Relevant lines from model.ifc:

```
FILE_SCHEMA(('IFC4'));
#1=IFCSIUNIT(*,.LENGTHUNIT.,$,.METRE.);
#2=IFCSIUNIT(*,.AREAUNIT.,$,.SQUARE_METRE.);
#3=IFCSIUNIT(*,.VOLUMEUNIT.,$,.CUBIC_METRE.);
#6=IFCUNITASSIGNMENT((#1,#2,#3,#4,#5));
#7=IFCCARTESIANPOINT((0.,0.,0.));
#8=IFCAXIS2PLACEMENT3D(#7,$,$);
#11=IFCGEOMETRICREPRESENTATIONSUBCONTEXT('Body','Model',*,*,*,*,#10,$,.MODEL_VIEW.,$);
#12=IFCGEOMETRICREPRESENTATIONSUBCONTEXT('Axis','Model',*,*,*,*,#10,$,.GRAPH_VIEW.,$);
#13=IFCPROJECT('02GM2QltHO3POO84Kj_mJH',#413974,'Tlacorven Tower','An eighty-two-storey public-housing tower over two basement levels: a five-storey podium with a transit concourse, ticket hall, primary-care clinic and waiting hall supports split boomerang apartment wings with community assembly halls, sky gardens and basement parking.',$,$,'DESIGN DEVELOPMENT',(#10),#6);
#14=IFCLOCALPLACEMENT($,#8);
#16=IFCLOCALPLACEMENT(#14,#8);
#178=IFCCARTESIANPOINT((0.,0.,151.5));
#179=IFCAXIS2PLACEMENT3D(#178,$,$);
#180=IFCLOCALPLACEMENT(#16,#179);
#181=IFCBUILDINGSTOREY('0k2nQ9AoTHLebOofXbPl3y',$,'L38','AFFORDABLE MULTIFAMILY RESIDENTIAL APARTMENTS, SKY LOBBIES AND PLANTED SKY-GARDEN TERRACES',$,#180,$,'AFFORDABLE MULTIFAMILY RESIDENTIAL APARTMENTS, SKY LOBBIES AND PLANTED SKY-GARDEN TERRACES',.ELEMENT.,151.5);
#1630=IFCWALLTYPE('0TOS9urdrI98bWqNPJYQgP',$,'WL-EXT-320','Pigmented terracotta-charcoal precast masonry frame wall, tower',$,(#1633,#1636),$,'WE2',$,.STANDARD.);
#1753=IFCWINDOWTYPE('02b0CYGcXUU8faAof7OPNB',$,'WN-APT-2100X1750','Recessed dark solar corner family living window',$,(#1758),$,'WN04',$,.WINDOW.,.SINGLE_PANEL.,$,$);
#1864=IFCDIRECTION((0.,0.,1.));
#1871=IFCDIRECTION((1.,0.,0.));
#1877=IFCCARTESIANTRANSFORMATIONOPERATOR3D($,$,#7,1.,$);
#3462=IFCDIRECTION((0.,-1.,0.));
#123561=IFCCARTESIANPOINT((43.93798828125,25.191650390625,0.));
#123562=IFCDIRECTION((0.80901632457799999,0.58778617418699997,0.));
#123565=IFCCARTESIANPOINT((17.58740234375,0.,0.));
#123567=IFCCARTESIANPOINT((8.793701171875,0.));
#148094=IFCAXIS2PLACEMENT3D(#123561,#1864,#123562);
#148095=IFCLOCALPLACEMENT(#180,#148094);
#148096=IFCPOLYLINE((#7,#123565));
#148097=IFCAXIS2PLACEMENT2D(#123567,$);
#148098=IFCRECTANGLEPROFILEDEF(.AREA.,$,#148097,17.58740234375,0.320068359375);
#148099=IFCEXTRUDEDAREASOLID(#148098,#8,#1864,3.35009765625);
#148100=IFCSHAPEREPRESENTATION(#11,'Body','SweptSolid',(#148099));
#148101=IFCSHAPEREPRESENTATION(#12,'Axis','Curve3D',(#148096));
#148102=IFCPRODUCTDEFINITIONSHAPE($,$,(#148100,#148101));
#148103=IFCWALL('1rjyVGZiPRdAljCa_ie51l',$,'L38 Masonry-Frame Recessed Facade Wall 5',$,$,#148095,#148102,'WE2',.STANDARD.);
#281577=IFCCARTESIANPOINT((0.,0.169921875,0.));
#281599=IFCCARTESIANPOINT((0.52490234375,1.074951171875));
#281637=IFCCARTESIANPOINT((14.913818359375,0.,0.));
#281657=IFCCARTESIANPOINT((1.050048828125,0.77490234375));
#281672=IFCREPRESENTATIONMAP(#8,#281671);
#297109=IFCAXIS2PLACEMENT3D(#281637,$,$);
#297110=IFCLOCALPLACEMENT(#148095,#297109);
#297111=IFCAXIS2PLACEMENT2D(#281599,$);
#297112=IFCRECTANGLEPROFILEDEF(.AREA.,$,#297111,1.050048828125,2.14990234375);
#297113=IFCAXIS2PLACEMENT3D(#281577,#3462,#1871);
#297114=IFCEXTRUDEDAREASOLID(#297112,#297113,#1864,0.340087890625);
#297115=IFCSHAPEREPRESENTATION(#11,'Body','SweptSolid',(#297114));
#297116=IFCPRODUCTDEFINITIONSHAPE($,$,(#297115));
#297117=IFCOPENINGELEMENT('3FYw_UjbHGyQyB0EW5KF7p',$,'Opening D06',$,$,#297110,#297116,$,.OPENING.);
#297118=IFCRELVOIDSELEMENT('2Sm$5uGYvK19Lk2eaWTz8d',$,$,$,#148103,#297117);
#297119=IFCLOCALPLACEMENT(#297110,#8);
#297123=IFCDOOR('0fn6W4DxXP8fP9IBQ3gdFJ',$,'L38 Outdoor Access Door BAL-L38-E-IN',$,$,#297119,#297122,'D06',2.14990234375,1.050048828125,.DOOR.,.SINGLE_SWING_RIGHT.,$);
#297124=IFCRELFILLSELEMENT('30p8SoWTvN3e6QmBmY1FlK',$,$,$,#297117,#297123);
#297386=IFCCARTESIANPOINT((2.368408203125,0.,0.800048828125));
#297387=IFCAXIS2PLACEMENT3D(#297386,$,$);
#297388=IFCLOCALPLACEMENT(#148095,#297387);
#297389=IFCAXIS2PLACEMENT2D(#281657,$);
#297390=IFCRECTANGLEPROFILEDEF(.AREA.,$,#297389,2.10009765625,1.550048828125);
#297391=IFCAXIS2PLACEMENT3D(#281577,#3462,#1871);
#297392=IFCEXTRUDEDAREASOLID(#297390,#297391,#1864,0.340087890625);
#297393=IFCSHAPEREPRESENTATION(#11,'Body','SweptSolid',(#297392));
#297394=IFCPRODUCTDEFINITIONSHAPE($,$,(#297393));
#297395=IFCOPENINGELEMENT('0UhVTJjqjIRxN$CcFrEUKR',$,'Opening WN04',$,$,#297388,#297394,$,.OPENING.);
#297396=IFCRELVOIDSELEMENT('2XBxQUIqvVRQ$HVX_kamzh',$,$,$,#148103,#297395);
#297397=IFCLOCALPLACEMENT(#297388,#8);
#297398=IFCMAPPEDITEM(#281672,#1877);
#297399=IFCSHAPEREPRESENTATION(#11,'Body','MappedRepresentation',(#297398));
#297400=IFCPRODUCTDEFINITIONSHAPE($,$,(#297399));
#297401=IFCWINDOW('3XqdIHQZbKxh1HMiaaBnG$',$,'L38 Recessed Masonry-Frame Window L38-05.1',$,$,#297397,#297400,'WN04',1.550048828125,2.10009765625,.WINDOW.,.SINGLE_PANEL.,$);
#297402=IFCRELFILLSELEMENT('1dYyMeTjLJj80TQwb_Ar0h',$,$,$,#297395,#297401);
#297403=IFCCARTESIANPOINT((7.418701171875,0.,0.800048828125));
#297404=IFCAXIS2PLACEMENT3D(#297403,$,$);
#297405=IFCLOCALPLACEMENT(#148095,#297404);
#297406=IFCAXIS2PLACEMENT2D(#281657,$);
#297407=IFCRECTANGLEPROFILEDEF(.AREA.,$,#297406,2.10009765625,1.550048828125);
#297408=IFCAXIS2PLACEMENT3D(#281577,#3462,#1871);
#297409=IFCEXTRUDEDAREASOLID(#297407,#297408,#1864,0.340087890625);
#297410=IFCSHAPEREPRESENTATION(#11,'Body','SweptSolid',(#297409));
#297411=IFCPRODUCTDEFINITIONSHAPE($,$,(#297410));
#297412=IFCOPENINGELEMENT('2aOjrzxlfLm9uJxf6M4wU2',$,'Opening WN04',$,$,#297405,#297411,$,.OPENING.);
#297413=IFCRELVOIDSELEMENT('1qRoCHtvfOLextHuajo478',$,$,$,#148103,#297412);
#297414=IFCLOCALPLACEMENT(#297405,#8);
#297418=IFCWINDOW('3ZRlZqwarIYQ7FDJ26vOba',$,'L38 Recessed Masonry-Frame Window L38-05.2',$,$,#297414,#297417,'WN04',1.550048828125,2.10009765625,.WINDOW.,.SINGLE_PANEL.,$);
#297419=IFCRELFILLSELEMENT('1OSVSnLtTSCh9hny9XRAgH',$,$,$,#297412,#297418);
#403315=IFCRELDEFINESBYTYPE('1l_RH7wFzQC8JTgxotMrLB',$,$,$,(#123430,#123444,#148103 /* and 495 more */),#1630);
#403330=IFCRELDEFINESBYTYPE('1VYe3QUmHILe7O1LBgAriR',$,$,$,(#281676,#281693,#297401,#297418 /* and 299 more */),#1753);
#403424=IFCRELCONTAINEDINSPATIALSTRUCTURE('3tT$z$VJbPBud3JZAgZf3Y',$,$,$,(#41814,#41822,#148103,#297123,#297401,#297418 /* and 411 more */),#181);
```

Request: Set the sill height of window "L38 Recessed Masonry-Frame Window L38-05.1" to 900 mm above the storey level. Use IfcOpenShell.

```python
import numpy as np
import ifcopenshell
import ifcopenshell.api.geometry
import ifcopenshell.geom
import ifcopenshell.util.element
import ifcopenshell.util.placement
import ifcopenshell.util.shape
import ifcopenshell.util.unit

model = ifcopenshell.open("model.ifc")
unit_scale = ifcopenshell.util.unit.calculate_unit_scale(model)

window = model.by_guid("3XqdIHQZbKxh1HMiaaBnG$")
opening = window.FillsVoids[0].RelatingOpeningElement
storey = ifcopenshell.util.element.get_container(window, ifc_class="IfcBuildingStorey")
level = ifcopenshell.util.placement.get_local_placement(storey.ObjectPlacement)[2, 3]

# The opening's origin need not be at the sill, so measure its lowest point.
shape = ifcopenshell.geom.create_shape(ifcopenshell.geom.settings(), opening)
bottom = ifcopenshell.util.shape.get_shape_bottom_elevation(shape, shape.geometry) / unit_scale
dz = level + 0.9 / unit_scale - bottom

shift = np.array([0.0, 0.0, dz])
# The window is placed relative to its opening, so it follows when the opening moves.
matrix = ifcopenshell.util.placement.get_local_placement(opening.ObjectPlacement)
matrix[:3, 3] += shift
ifcopenshell.api.geometry.edit_object_placement(
    model, product=opening, matrix=matrix, is_si=False, should_transform_children=True
)

print(f"moved by {dz * unit_scale:+.3f} m")

model.write("model-out.ifc")
```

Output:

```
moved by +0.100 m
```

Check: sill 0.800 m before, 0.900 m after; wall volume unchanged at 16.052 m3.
